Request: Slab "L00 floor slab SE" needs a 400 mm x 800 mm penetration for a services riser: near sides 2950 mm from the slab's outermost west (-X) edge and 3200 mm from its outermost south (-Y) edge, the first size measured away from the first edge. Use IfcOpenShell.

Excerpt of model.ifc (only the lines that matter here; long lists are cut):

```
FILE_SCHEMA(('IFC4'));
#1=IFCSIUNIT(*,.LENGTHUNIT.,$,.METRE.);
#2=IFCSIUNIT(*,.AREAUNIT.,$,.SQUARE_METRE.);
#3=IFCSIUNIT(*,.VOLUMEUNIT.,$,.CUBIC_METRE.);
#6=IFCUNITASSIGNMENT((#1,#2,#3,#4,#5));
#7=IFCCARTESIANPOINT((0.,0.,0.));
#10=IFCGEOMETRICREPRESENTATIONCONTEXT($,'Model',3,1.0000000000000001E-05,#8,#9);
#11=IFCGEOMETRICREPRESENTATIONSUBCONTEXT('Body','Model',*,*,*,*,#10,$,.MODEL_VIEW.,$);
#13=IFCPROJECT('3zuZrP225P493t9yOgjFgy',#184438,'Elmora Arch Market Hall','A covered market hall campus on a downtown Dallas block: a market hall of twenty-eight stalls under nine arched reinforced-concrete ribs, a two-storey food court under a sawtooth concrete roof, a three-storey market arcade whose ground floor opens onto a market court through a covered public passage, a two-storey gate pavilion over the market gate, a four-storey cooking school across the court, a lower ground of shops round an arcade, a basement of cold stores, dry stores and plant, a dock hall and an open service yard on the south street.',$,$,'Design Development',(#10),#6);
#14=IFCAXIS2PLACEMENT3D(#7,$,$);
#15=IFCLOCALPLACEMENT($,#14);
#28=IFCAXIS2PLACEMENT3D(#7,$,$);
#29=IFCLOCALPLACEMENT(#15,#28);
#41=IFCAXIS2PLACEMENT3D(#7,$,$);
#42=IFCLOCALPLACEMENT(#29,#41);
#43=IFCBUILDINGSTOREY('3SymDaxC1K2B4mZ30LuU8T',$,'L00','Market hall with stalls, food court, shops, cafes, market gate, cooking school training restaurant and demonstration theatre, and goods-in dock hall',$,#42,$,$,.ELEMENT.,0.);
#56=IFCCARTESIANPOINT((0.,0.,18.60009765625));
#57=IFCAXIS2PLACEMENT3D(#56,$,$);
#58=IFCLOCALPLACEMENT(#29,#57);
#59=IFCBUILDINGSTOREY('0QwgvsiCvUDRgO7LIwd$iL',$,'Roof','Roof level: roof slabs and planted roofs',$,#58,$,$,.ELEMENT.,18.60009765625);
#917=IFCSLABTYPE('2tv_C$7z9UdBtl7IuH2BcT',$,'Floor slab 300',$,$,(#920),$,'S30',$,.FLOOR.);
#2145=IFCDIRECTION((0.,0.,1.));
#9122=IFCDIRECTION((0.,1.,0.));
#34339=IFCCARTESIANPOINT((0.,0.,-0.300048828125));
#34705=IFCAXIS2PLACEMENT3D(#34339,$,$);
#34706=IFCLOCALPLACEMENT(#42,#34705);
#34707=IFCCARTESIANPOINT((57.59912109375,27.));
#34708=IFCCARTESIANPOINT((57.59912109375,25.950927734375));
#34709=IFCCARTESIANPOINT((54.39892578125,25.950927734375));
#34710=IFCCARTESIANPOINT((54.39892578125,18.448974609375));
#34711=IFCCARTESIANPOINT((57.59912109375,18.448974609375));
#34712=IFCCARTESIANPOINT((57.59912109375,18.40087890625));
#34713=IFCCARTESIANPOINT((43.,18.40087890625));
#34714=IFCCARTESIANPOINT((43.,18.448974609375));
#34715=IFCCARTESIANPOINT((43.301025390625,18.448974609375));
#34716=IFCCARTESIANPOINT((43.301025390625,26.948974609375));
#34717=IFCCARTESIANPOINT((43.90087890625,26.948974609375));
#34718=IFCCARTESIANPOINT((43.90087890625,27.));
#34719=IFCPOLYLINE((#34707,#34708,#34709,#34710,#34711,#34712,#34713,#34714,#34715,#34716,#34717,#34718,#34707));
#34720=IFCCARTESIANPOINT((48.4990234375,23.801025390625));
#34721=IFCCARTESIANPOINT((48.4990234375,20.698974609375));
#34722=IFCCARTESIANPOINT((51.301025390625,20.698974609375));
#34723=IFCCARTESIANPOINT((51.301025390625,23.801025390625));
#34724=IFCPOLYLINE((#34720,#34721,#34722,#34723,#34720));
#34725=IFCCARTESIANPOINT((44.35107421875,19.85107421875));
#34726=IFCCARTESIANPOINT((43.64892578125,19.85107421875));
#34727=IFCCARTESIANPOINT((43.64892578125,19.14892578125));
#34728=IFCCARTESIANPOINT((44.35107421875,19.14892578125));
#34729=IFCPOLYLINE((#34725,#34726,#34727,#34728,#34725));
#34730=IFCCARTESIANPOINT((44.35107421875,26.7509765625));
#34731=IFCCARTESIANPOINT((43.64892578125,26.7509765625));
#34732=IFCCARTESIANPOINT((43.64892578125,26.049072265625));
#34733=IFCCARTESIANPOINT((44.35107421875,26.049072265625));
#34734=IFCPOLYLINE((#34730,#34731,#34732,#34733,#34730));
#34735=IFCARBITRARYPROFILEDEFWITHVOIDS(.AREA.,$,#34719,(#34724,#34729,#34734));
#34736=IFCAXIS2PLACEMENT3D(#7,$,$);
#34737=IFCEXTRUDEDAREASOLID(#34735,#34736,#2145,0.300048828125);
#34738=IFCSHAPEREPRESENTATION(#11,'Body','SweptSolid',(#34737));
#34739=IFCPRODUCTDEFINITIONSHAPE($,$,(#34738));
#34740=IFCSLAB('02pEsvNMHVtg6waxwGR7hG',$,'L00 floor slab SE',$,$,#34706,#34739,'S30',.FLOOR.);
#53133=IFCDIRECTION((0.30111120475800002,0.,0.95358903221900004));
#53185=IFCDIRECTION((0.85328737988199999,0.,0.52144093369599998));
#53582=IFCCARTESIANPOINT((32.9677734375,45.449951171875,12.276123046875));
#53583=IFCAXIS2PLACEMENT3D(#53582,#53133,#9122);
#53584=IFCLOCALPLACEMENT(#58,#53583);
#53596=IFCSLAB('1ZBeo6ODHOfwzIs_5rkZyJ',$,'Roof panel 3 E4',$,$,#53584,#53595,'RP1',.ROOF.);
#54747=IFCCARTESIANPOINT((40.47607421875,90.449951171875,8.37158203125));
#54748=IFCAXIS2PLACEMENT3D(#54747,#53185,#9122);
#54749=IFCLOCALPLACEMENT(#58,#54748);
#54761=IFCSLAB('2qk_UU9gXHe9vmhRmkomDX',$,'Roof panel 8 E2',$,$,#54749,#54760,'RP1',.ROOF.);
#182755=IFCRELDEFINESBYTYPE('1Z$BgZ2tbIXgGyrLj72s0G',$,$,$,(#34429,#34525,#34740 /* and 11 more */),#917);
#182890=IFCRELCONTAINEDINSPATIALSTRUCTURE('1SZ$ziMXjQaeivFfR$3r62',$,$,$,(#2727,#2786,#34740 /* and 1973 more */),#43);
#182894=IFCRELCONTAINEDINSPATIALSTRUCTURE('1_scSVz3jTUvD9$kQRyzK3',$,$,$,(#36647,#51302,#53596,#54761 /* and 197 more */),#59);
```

```python
import numpy as np
import ifcopenshell
import ifcopenshell.api.feature
import ifcopenshell.api.geometry
import ifcopenshell.api.root
import ifcopenshell.geom
import ifcopenshell.util.placement
import ifcopenshell.util.representation
import ifcopenshell.util.shape
import ifcopenshell.util.unit

model = ifcopenshell.open("model.ifc")
unit_scale = ifcopenshell.util.unit.calculate_unit_scale(model)
settings = ifcopenshell.geom.settings()


def volume(element):
    """Net volume in cubic metres, openings subtracted."""
    shape = ifcopenshell.geom.create_shape(settings, element)
    return ifcopenshell.util.shape.get_volume(shape.geometry)


slab = model.by_guid("02pEsvNMHVtg6waxwGR7hG")
before = volume(slab)

# Extent in the slab's own axes, in metres. The edges named are its -X and -Y sides.
slab_shape = ifcopenshell.geom.create_shape(settings, slab)
vertices = ifcopenshell.util.shape.get_vertices(slab_shape.geometry)
x_min, y_min, bottom = vertices.min(axis=0)
top = vertices[:, 2].max()

opening = ifcopenshell.api.root.create_entity(model, ifc_class="IfcOpeningElement", name="Services riser opening", predefined_type="OPENING")
context = ifcopenshell.util.representation.get_context(model, "Model", "Body", "MODEL_VIEW")
width, depth = 0.4, 0.8
outline = [(0.0, 0.0), (width, 0.0), (width, depth), (0.0, depth), (0.0, 0.0)]
# Overshoot both faces by 50 mm so the cut is clean.
shape = ifcopenshell.api.geometry.add_slab_representation(
    model, context=context, depth=top - bottom + 0.1, polyline=outline
)
ifcopenshell.api.geometry.assign_representation(model, product=opening, representation=shape)

matrix = ifcopenshell.util.placement.get_local_placement(slab.ObjectPlacement)
matrix[:, 3] = matrix @ np.append(np.array([x_min + 2.95, y_min + 3.2, bottom - 0.05]) / unit_scale, 1.0)
ifcopenshell.api.geometry.edit_object_placement(model, product=opening, matrix=matrix, is_si=False)
ifcopenshell.api.feature.add_feature(model, feature=opening, element=slab)

after = volume(slab)

print(f"slab volume {before:.3f} -> {after:.3f} m3")

model.write("model_rev.ifc")
```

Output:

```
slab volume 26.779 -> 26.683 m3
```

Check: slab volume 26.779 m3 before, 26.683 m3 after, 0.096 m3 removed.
